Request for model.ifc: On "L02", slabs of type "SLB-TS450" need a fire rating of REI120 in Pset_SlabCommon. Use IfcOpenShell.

First a look at what the model holds.

```python
import ifcopenshell
import ifcopenshell.util.element

model = ifcopenshell.open("model.ifc")
print(model.schema)
storey = next(s for s in model.by_type("IfcBuildingStorey") if s.Name == "L02")
slabs = [e for e in ifcopenshell.util.element.get_decomposition(storey) if e.is_a("IfcSlab")]
seen = {}
for e in slabs:
    element_type = ifcopenshell.util.element.get_type(e)
    key = (element_type.Name if element_type != e and element_type else None, ifcopenshell.util.element.get_pset(e, "Pset_SlabCommon", "FireRating"))
    seen[key] = seen.get(key, 0) + 1
for (name, value), count in sorted(seen.items(), key=str):
    print(count, "x", name, "|", value)
```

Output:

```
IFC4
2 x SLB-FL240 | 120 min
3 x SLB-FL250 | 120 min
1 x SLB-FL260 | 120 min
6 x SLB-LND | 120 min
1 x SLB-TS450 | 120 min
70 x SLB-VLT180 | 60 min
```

```python
import ifcopenshell
import ifcopenshell.api.pset
import ifcopenshell.util.element

model = ifcopenshell.open("model.ifc")

storey = next(s for s in model.by_type("IfcBuildingStorey") if s.Name == "L02")
slabs = [e for e in ifcopenshell.util.element.get_decomposition(storey) if e.is_a("IfcSlab")]

count = 0
for e in slabs:
    element_type = ifcopenshell.util.element.get_type(e)
    if element_type in (None, e) or element_type.Name != "SLB-TS450":
        continue
    # add_pset returns the element's existing set when there is one.
    pset = ifcopenshell.api.pset.add_pset(model, product=e, name="Pset_SlabCommon")
    ifcopenshell.api.pset.edit_pset(model, pset=pset, properties={"FireRating": "REI120"})
    count += 1

print(count, "slabs updated")

model.write("model_v2.ifc")
```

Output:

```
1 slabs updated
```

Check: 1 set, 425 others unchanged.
